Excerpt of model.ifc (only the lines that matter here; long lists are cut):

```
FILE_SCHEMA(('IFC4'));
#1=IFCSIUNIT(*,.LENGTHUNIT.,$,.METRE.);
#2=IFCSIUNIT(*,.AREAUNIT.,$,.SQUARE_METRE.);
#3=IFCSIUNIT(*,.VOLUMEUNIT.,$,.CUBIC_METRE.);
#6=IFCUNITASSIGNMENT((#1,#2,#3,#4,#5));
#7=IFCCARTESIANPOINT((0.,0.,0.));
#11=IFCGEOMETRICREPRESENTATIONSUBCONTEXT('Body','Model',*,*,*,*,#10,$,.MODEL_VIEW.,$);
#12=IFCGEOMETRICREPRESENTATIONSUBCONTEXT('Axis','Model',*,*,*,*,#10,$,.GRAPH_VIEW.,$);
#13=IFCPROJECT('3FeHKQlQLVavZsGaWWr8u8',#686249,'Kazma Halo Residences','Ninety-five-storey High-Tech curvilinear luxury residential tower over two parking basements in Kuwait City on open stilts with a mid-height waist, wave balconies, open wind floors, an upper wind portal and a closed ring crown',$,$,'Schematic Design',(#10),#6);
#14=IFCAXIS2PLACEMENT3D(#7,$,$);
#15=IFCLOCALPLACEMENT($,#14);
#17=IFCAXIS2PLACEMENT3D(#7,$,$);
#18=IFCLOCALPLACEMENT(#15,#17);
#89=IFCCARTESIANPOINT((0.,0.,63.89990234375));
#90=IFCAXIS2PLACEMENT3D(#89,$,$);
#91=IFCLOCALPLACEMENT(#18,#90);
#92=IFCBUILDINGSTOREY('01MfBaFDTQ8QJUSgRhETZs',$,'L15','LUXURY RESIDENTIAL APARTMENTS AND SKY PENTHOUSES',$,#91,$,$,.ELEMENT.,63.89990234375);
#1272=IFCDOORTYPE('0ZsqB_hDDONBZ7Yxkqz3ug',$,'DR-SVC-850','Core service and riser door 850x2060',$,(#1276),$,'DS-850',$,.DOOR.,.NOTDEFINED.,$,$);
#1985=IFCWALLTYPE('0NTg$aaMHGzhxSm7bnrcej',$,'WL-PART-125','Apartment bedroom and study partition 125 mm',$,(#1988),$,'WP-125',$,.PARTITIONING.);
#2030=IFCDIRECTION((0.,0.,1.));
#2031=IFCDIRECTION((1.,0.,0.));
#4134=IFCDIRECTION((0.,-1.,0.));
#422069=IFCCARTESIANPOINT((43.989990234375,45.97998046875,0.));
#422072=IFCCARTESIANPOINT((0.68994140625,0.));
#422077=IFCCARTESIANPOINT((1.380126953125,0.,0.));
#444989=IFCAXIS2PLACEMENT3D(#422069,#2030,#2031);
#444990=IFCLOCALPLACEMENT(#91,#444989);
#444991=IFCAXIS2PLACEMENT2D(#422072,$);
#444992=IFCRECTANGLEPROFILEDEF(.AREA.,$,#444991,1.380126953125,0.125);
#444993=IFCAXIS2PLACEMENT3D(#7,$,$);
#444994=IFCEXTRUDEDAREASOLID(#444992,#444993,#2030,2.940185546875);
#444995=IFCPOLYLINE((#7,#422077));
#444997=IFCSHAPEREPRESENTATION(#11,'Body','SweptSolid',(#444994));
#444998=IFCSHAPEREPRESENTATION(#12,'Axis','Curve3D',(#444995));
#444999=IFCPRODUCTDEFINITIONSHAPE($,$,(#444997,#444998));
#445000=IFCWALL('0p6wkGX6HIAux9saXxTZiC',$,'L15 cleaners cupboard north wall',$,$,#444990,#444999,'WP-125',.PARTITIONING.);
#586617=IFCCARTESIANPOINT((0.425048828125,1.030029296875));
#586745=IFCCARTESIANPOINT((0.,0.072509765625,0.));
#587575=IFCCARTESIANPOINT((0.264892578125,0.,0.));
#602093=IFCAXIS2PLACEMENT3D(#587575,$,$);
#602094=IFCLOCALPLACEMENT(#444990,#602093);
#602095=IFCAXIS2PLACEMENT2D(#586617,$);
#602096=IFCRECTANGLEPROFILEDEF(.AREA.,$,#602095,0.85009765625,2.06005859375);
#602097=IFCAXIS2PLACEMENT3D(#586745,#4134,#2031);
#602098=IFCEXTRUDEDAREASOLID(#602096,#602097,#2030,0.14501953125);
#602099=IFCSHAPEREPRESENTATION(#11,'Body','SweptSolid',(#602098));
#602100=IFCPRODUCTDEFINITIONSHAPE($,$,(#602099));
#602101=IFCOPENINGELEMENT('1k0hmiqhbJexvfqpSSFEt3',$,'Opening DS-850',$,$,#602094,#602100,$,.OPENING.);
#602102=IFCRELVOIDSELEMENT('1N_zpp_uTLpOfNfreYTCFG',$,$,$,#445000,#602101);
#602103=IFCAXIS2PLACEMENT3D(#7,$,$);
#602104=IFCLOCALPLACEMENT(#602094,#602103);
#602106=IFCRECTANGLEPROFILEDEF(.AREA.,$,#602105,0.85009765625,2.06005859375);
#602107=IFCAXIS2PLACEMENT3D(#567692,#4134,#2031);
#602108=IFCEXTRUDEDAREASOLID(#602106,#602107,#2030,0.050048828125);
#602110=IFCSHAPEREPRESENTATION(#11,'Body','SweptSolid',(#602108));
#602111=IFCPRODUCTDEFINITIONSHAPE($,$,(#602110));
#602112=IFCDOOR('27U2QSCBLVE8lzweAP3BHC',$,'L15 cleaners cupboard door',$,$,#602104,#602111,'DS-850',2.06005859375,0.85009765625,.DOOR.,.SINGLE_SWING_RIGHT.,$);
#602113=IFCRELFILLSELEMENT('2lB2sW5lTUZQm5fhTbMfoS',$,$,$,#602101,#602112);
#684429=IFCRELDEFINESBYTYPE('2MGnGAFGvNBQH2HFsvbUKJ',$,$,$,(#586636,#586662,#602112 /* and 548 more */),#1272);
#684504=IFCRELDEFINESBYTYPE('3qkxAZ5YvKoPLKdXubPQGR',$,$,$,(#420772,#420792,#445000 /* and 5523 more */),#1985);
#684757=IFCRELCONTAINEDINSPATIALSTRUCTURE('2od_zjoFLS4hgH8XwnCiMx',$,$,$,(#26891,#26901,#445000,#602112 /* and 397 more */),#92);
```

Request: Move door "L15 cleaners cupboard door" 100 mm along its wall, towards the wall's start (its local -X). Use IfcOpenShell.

```python
import ifcopenshell
import ifcopenshell.api.geometry
import ifcopenshell.util.placement

model = ifcopenshell.open("model.ifc")

door = model.by_guid("27U2QSCBLVE8lzweAP3BHC")
opening = door.FillsVoids[0].RelatingOpeningElement
wall = opening.VoidsElements[0].RelatingBuildingElement

wall_matrix = ifcopenshell.util.placement.get_local_placement(wall.ObjectPlacement)
shift = wall_matrix[:3, 0] * -0.1
before = ifcopenshell.util.placement.get_local_placement(door.ObjectPlacement)[:3, 3].copy()

# The door is placed relative to its opening, so it follows when the opening moves.
matrix = ifcopenshell.util.placement.get_local_placement(opening.ObjectPlacement)
matrix[:3, 3] += shift
ifcopenshell.api.geometry.edit_object_placement(
    model, product=opening, matrix=matrix, is_si=False, should_transform_children=True
)

after = ifcopenshell.util.placement.get_local_placement(door.ObjectPlacement)[:3, 3]
print("door moved by", (after - before).round(3) + 0.0)

model.write("model-out.ifc")
```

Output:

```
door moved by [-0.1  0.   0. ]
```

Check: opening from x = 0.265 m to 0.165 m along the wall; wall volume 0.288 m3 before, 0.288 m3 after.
